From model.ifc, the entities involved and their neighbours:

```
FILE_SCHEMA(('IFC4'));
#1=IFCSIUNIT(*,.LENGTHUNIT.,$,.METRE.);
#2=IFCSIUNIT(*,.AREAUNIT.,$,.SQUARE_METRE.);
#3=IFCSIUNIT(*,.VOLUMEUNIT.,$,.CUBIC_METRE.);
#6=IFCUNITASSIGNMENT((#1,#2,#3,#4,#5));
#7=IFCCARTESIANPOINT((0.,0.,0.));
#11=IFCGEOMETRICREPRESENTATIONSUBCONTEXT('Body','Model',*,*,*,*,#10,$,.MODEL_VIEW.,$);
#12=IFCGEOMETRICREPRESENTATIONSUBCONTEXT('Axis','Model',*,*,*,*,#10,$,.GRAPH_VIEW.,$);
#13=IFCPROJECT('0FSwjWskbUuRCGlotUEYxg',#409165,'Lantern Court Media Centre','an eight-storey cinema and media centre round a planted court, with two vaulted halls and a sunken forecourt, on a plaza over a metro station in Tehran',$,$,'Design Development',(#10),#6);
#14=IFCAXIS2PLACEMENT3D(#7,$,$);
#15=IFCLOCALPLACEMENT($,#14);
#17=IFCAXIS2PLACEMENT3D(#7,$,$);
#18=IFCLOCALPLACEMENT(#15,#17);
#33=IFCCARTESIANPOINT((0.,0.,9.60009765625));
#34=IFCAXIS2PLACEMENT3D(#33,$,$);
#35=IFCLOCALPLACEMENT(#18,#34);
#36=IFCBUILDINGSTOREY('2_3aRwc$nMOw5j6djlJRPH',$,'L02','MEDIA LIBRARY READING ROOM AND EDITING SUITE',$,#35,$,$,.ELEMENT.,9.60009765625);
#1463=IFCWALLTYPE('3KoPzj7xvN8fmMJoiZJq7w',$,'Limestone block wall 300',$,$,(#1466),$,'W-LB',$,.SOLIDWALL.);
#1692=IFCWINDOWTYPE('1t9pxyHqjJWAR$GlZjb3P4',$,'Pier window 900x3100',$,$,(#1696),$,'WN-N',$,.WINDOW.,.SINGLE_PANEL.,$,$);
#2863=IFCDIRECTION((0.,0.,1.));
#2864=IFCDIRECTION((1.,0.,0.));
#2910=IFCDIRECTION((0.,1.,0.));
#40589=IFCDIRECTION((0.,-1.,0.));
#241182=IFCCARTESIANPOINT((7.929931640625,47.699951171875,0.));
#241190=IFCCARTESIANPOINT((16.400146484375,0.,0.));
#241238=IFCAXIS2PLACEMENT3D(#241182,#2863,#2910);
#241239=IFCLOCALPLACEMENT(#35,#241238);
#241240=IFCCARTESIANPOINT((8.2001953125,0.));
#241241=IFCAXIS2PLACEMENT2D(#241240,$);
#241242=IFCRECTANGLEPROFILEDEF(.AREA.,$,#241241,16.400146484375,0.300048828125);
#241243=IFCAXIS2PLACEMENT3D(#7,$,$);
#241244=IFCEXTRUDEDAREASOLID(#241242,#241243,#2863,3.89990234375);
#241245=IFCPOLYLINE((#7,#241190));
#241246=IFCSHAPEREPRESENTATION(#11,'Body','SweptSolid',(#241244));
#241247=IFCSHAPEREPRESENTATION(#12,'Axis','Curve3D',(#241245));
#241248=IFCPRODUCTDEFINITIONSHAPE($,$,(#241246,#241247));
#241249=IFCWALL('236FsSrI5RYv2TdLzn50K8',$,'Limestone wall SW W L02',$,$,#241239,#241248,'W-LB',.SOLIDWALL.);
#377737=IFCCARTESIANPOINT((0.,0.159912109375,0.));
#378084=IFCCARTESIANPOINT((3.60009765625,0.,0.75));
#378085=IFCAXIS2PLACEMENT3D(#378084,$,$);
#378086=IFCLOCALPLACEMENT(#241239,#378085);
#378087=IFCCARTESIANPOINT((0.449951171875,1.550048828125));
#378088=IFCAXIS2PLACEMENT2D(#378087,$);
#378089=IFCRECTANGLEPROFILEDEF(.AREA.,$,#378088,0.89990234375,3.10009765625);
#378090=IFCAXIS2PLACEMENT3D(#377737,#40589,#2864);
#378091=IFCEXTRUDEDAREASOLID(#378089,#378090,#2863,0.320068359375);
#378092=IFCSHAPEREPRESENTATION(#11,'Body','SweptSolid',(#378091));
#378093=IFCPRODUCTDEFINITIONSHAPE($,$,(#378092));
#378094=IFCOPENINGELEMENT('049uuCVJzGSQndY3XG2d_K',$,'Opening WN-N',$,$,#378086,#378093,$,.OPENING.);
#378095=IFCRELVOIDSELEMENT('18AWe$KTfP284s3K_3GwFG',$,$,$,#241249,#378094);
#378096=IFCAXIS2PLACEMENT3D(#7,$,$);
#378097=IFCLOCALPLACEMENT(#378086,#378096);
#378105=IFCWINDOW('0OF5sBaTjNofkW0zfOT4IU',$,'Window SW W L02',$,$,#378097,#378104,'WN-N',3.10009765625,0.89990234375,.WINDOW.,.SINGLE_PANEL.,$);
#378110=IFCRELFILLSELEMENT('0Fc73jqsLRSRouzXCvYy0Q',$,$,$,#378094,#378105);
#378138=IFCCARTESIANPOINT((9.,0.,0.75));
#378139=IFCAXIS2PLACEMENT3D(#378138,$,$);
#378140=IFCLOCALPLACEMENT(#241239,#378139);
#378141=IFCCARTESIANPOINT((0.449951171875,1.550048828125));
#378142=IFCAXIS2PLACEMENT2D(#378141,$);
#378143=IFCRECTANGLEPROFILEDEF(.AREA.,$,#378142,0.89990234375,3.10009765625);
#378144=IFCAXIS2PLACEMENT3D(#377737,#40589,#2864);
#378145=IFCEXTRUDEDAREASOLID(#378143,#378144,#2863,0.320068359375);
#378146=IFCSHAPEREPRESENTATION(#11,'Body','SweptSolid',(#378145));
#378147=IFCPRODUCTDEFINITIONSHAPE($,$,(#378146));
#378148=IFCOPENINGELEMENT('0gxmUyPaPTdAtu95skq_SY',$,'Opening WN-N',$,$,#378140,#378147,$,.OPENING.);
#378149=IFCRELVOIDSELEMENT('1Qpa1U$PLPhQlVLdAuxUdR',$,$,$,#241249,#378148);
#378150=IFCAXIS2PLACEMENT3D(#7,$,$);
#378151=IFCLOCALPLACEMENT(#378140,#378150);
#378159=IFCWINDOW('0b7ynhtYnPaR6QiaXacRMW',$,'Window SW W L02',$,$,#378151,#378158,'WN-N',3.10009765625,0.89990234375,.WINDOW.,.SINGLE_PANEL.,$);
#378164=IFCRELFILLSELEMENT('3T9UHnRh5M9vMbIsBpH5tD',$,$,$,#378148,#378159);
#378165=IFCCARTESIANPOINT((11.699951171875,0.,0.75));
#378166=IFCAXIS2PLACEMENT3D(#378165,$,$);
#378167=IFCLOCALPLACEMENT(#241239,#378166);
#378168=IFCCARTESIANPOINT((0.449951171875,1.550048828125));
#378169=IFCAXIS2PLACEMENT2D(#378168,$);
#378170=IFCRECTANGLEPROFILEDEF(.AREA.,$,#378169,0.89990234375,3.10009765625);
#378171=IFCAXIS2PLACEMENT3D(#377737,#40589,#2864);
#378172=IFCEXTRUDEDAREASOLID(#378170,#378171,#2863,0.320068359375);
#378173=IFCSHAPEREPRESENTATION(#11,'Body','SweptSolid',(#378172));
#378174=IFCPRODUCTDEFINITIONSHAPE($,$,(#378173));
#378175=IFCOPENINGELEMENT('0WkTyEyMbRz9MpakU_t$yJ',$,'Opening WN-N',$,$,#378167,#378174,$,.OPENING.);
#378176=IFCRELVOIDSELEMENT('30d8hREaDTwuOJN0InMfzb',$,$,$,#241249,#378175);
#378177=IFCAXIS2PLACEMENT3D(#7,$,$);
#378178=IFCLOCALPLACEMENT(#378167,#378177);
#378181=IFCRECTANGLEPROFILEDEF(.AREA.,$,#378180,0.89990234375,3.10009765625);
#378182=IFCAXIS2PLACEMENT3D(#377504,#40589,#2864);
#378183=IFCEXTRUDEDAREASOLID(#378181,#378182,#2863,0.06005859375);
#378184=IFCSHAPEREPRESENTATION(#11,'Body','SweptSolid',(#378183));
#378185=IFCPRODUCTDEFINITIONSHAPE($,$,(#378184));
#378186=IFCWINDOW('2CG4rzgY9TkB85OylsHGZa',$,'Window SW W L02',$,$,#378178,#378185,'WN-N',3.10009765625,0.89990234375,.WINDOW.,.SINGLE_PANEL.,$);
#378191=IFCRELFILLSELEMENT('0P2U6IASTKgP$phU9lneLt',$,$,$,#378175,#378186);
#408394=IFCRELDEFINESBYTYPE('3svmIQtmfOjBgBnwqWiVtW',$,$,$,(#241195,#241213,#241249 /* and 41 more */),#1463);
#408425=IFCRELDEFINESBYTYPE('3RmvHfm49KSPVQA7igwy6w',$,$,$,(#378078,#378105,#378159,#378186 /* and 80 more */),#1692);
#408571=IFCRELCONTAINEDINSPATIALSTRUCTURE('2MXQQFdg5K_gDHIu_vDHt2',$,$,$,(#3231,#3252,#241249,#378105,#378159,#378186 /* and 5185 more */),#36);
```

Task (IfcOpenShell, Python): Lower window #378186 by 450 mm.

```python
import numpy as np
import ifcopenshell
import ifcopenshell.api.geometry
import ifcopenshell.util.placement
import ifcopenshell.util.unit

model = ifcopenshell.open("model.ifc")
unit_scale = ifcopenshell.util.unit.calculate_unit_scale(model)

window = model.by_id(378186)
opening = window.FillsVoids[0].RelatingOpeningElement
dz = -0.45 / unit_scale

shift = np.array([0.0, 0.0, dz])
# The window is placed relative to its opening, so it follows when the opening moves.
matrix = ifcopenshell.util.placement.get_local_placement(opening.ObjectPlacement)
matrix[:3, 3] += shift
ifcopenshell.api.geometry.edit_object_placement(
    model, product=opening, matrix=matrix, is_si=False, should_transform_children=True
)

print(f"moved by {dz * unit_scale:+.3f} m")

model.write("model_v2.ifc")
```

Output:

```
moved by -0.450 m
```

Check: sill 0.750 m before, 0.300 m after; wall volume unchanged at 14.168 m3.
